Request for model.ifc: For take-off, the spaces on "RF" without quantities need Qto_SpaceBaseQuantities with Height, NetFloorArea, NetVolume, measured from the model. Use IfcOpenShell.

First a look at what the model holds.

```python
import ifcopenshell
import ifcopenshell.util.element
import ifcopenshell.util.unit

model = ifcopenshell.open("model.ifc")
print(model.schema)
for unit_type in ("LENGTHUNIT", "AREAUNIT", "VOLUMEUNIT"):
    print(unit_type, ifcopenshell.util.unit.calculate_unit_scale(model, unit_type))
storey = next(s for s in model.by_type("IfcBuildingStorey") if s.Name == "RF")
spaces = [e for e in ifcopenshell.util.element.get_decomposition(storey) if e.is_a("IfcSpace")]
for e in sorted(spaces, key=lambda e: e.id()):
    print(e.id(), e.is_a(), e.Name, list(ifcopenshell.util.element.get_psets(e, qtos_only=True)), sep=" | ")
```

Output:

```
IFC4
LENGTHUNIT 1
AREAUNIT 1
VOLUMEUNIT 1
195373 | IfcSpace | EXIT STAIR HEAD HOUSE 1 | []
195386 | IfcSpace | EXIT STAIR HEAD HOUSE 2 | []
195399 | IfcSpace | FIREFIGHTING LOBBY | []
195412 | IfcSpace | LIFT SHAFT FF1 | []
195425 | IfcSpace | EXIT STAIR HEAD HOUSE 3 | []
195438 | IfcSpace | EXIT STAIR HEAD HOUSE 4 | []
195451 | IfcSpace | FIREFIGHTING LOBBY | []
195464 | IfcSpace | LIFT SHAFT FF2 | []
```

```python
import ifcopenshell
import ifcopenshell.api.pset
import ifcopenshell.geom
import ifcopenshell.util.element
import ifcopenshell.util.shape
import ifcopenshell.util.unit

model = ifcopenshell.open("model.ifc")
unit_scale = ifcopenshell.util.unit.calculate_unit_scale(model)
area_scale = ifcopenshell.util.unit.calculate_unit_scale(model, "AREAUNIT")
volume_scale = ifcopenshell.util.unit.calculate_unit_scale(model, "VOLUMEUNIT")
settings = ifcopenshell.geom.settings()

storey = next(s for s in model.by_type("IfcBuildingStorey") if s.Name == "RF")
spaces = [e for e in ifcopenshell.util.element.get_decomposition(storey) if e.is_a("IfcSpace")]

for e in sorted(spaces, key=lambda e: e.id()):
    if ifcopenshell.util.element.get_psets(e, qtos_only=True, should_inherit=False):
        continue
    # Geometry comes back in metres, in the element's own axes.
    shape = ifcopenshell.geom.create_shape(settings, e)
    values = {
        "Height": ifcopenshell.util.shape.get_z(shape.geometry) / unit_scale,
        "NetFloorArea": ifcopenshell.util.shape.get_footprint_area(shape.geometry) / area_scale,
        "NetVolume": ifcopenshell.util.shape.get_volume(shape.geometry) / volume_scale,
    }
    qto = ifcopenshell.api.pset.add_qto(model, product=e, name="Qto_SpaceBaseQuantities")
    ifcopenshell.api.pset.edit_qto(model, qto=qto, properties=values)
    print(e.id(), {k: round(v, 3) for k, v in values.items()})

model.write("model_edited.ifc")
```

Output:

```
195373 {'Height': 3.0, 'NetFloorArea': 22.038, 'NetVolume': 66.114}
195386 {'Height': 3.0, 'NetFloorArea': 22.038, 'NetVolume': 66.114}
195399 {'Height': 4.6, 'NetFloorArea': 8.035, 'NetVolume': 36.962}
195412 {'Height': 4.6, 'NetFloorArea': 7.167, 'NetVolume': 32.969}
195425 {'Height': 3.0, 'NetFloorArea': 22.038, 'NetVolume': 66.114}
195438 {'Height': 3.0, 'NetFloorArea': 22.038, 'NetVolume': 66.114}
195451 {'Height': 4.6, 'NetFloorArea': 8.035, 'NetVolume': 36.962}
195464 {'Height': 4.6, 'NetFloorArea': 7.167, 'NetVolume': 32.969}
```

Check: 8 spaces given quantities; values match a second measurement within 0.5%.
